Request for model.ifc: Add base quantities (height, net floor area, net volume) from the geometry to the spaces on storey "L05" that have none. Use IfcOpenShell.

First a look at what the model holds.

```python
import ifcopenshell
import ifcopenshell.util.element
import ifcopenshell.util.unit

model = ifcopenshell.open("model.ifc")
print(model.schema)
for unit_type in ("LENGTHUNIT", "AREAUNIT", "VOLUMEUNIT"):
    print(unit_type, ifcopenshell.util.unit.calculate_unit_scale(model, unit_type))
storey = next(s for s in model.by_type("IfcBuildingStorey") if s.Name == "L05")
spaces = [e for e in ifcopenshell.util.element.get_decomposition(storey) if e.is_a("IfcSpace")]
for e in sorted(spaces, key=lambda e: e.id()):
    print(e.id(), e.is_a(), e.Name, list(ifcopenshell.util.element.get_psets(e, qtos_only=True)), sep=" | ")
```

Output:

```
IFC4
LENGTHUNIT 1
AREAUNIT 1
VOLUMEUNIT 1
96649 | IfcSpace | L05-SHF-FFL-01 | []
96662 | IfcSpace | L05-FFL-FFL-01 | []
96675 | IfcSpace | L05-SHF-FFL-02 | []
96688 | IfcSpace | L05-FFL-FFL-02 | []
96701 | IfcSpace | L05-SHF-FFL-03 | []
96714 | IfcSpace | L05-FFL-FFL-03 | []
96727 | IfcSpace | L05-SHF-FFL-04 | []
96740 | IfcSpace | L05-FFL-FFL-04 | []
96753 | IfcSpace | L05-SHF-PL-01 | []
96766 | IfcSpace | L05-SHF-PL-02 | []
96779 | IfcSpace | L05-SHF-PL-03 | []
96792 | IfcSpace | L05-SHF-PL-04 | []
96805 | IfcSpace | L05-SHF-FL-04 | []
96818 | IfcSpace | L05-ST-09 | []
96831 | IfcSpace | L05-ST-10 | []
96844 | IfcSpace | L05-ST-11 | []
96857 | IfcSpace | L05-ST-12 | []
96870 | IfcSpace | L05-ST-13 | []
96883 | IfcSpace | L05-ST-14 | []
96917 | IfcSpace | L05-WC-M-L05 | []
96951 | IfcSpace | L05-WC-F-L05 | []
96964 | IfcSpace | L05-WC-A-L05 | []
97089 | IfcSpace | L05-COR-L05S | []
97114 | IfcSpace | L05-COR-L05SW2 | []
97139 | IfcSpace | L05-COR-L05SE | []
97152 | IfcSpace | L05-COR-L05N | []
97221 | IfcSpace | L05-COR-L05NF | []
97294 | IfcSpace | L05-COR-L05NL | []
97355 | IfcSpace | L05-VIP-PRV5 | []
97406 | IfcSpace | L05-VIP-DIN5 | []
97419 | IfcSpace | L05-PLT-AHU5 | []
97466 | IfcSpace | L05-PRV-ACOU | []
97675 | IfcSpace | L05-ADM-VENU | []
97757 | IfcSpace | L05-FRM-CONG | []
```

```python
import ifcopenshell
import ifcopenshell.api.pset
import ifcopenshell.geom
import ifcopenshell.util.element
import ifcopenshell.util.shape
import ifcopenshell.util.unit

model = ifcopenshell.open("model.ifc")
unit_scale = ifcopenshell.util.unit.calculate_unit_scale(model)
area_scale = ifcopenshell.util.unit.calculate_unit_scale(model, "AREAUNIT")
volume_scale = ifcopenshell.util.unit.calculate_unit_scale(model, "VOLUMEUNIT")
settings = ifcopenshell.geom.settings()

storey = next(s for s in model.by_type("IfcBuildingStorey") if s.Name == "L05")
spaces = [e for e in ifcopenshell.util.element.get_decomposition(storey) if e.is_a("IfcSpace")]

for e in sorted(spaces, key=lambda e: e.id()):
    if ifcopenshell.util.element.get_psets(e, qtos_only=True, should_inherit=False):
        continue
    # Geometry comes back in metres, in the element's own axes.
    shape = ifcopenshell.geom.create_shape(settings, e)
    values = {
        "Height": ifcopenshell.util.shape.get_z(shape.geometry) / unit_scale,
        "NetFloorArea": ifcopenshell.util.shape.get_footprint_area(shape.geometry) / area_scale,
        "NetVolume": ifcopenshell.util.shape.get_volume(shape.geometry) / volume_scale,
    }
    qto = ifcopenshell.api.pset.add_qto(model, product=e, name="Qto_SpaceBaseQuantities")
    ifcopenshell.api.pset.edit_qto(model, qto=qto, properties=values)
    print(e.id(), {k: round(v, 3) for k, v in values.items()})

model.write("model_updated.ifc")
```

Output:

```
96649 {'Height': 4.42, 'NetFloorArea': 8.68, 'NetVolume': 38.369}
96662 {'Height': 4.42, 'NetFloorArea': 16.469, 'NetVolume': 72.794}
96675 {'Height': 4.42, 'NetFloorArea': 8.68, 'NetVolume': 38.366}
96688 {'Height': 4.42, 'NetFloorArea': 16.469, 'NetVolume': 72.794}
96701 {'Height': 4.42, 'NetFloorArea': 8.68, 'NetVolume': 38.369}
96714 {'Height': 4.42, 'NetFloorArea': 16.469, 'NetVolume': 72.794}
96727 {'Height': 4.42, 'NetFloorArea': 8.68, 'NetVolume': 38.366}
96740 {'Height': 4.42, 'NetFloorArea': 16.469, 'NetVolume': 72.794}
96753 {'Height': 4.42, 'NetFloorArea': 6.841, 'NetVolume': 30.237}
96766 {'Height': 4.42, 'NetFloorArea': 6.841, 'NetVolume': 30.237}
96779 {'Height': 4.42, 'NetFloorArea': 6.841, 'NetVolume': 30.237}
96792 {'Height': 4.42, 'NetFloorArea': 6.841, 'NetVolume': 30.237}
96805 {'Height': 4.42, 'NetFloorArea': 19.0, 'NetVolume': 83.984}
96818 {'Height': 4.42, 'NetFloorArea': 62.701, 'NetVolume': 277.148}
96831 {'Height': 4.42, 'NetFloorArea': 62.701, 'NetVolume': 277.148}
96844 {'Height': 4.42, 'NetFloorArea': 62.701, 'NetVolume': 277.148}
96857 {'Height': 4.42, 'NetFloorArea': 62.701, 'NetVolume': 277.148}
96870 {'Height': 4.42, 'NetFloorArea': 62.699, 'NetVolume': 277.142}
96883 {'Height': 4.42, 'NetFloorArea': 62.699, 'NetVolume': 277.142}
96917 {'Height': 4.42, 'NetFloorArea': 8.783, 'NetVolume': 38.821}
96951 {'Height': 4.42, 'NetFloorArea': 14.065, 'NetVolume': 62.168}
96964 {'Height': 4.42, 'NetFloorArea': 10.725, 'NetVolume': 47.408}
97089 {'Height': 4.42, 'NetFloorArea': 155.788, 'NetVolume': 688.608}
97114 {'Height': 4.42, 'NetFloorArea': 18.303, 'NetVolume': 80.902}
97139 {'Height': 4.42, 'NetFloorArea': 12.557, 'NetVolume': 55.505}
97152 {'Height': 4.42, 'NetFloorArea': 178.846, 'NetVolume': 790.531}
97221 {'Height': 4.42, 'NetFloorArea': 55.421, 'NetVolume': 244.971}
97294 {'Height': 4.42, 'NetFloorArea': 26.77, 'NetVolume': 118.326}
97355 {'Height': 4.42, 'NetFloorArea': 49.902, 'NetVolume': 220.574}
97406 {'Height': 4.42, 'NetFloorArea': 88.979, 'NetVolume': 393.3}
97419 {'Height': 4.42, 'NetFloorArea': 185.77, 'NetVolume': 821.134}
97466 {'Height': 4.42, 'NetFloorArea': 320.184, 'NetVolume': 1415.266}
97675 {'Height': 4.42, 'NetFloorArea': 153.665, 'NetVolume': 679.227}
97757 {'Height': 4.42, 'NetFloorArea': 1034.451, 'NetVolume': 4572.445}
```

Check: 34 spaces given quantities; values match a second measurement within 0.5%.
